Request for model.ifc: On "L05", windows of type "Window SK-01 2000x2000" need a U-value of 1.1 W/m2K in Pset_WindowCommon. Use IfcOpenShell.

First a look at what the model holds.

```python
import ifcopenshell
import ifcopenshell.util.element

model = ifcopenshell.open("model.ifc")
print(model.schema)
storey = next(s for s in model.by_type("IfcBuildingStorey") if s.Name == "L05")
windows = [e for e in ifcopenshell.util.element.get_decomposition(storey) if e.is_a("IfcWindow")]
seen = {}
for e in windows:
    element_type = ifcopenshell.util.element.get_type(e)
    key = (element_type.Name if element_type != e and element_type else None, ifcopenshell.util.element.get_pset(e, "Pset_WindowCommon", "ThermalTransmittance"))
    seen[key] = seen.get(key, 0) + 1
for (name, value), count in sorted(seen.items(), key=str):
    print(count, "x", name, "|", value)
```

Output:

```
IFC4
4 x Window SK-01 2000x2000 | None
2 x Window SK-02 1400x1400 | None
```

```python
import ifcopenshell
import ifcopenshell.api.pset
import ifcopenshell.util.element

model = ifcopenshell.open("model.ifc")

storey = next(s for s in model.by_type("IfcBuildingStorey") if s.Name == "L05")
windows = [e for e in ifcopenshell.util.element.get_decomposition(storey) if e.is_a("IfcWindow")]

count = 0
for e in windows:
    element_type = ifcopenshell.util.element.get_type(e)
    if element_type in (None, e) or element_type.Name != "Window SK-01 2000x2000":
        continue
    # add_pset returns the element's existing set when there is one.
    pset = ifcopenshell.api.pset.add_pset(model, product=e, name="Pset_WindowCommon")
    ifcopenshell.api.pset.edit_pset(model, pset=pset, properties={"ThermalTransmittance": 1.1})
    count += 1

print(count, "windows updated")

model.write("model_updated.ifc")
```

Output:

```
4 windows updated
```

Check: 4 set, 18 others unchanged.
